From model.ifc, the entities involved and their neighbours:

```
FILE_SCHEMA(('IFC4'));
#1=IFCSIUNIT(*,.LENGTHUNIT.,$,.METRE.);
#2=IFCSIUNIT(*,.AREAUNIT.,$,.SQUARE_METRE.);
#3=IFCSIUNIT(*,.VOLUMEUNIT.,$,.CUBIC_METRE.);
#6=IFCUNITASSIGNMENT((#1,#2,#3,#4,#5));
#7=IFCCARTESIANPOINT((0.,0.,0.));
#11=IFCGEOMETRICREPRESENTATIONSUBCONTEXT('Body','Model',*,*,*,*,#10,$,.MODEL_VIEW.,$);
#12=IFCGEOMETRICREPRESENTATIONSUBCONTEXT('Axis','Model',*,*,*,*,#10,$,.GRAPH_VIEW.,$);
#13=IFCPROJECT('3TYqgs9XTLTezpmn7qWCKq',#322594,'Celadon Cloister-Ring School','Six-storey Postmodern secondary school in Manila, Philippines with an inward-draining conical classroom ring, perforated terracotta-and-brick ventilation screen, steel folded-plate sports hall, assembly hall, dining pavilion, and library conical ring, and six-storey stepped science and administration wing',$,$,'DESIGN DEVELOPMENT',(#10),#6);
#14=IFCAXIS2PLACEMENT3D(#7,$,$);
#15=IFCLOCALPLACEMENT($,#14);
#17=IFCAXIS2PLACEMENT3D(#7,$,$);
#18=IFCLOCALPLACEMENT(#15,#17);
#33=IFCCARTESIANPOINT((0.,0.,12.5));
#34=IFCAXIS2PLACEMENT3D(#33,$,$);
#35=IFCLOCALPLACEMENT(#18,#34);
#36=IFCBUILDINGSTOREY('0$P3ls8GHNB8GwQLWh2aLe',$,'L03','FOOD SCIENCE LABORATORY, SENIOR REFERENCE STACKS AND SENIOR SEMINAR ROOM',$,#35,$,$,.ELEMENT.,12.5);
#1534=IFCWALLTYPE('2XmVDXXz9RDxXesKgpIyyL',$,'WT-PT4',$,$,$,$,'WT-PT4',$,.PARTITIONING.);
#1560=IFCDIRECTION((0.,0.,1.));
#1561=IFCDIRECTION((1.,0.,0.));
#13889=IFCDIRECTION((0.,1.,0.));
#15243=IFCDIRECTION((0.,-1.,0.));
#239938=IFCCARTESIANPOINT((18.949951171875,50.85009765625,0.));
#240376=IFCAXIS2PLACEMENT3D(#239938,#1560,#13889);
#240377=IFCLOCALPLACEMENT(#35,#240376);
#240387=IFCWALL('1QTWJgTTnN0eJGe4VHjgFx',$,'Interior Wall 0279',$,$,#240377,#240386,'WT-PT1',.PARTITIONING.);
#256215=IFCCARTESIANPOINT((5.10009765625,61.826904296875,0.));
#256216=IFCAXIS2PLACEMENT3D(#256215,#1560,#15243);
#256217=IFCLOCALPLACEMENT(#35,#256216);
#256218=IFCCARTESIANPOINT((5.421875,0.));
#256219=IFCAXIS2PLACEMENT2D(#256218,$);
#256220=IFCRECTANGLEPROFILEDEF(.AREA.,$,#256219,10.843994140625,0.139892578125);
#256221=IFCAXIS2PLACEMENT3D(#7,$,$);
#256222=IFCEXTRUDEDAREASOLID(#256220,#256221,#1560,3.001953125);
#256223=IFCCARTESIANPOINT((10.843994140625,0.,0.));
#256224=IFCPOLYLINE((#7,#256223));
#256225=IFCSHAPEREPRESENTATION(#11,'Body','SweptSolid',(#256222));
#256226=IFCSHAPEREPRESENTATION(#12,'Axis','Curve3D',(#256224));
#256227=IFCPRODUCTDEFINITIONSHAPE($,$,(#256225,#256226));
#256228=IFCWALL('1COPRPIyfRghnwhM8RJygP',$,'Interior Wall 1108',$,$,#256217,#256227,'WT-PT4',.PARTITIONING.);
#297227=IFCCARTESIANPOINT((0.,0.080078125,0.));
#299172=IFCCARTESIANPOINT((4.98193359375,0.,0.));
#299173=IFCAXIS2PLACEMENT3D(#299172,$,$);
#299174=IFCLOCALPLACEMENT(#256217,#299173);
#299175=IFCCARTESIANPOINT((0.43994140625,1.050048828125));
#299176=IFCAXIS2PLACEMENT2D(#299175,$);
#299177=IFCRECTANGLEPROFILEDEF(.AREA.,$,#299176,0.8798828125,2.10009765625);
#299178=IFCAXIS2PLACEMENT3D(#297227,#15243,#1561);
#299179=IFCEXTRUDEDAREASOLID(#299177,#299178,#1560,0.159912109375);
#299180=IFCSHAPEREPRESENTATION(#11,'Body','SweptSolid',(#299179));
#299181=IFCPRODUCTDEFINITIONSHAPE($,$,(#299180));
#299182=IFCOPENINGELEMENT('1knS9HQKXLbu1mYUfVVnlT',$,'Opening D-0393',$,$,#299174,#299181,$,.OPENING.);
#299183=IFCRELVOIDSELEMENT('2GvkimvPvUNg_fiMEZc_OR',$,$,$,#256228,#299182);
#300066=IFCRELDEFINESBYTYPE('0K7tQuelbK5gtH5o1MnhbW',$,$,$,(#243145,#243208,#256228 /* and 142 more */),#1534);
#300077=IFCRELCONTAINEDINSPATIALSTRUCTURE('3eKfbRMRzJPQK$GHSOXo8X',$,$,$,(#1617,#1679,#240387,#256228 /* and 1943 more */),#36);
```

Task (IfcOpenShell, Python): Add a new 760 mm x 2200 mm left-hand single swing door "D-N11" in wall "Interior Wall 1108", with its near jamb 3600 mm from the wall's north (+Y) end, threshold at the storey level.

```python
import numpy as np
import ifcopenshell
import ifcopenshell.api.feature
import ifcopenshell.api.geometry
import ifcopenshell.api.root
import ifcopenshell.api.spatial
import ifcopenshell.geom
import ifcopenshell.util.element
import ifcopenshell.util.placement
import ifcopenshell.util.representation
import ifcopenshell.util.shape
import ifcopenshell.util.unit

model = ifcopenshell.open("model.ifc")
unit_scale = ifcopenshell.util.unit.calculate_unit_scale(model)
settings = ifcopenshell.geom.settings()


def volume(element):
    """Net volume in cubic metres, openings subtracted."""
    shape = ifcopenshell.geom.create_shape(settings, element)
    return ifcopenshell.util.shape.get_volume(shape.geometry)


wall = model.by_guid("1COPRPIyfRghnwhM8RJygP")
storey = ifcopenshell.util.element.get_container(wall, ifc_class="IfcBuildingStorey")
context = ifcopenshell.util.representation.get_context(model, "Model", "Body", "MODEL_VIEW")
before = volume(wall)

width, height, from_end, sill = 0.76, 2.2, 3.6, 0.0  # metres

# The wall runs along its own X axis, and the end named is its -X end.
wall_shape = ifcopenshell.geom.create_shape(settings, wall)
x, y, z = ifcopenshell.util.shape.get_vertices(wall_shape.geometry).T
start = x.min() + from_end
face, thickness = float(y.min()), float(y.max() - y.min())
wall_matrix = ifcopenshell.util.placement.get_local_placement(wall.ObjectPlacement)
level = ifcopenshell.util.placement.get_local_placement(storey.ObjectPlacement)[2, 3]


def in_wall(x, y):
    """Placement at x, y metres in the wall's axes, at sill height."""
    matrix = wall_matrix.copy()
    matrix[:, 3] = wall_matrix @ np.array([x / unit_scale, y / unit_scale, 0.0, 1.0])
    matrix[2, 3] = level + sill / unit_scale
    return matrix


# Opening: a box that overshoots both wall faces by 50 mm.
opening = ifcopenshell.api.root.create_entity(model, ifc_class="IfcOpeningElement", predefined_type="OPENING")
box = ifcopenshell.api.geometry.add_wall_representation(
    model, context=context, length=width, height=height, thickness=thickness + 0.1
)
ifcopenshell.api.geometry.assign_representation(model, product=opening, representation=box)
ifcopenshell.api.geometry.edit_object_placement(model, product=opening, matrix=in_wall(start, face - 0.05), is_si=False)
ifcopenshell.api.feature.add_feature(model, feature=opening, element=wall)

door = ifcopenshell.api.root.create_entity(model, ifc_class="IfcDoor", name="D-N11", predefined_type="DOOR")
door.OverallWidth, door.OverallHeight = width / unit_scale, height / unit_scale
door.OperationType = "SINGLE_SWING_LEFT"
body = ifcopenshell.api.geometry.add_door_representation(
    model,
    context=context,
    overall_width=door.OverallWidth,
    overall_height=door.OverallHeight,
    operation_type="SINGLE_SWING_LEFT",
    lining_properties={"LiningDepth": thickness / unit_scale, "ThresholdDepth": thickness / unit_scale},
)
ifcopenshell.api.geometry.assign_representation(model, product=door, representation=body)
ifcopenshell.api.spatial.assign_container(model, products=[door], relating_structure=storey)
ifcopenshell.api.feature.add_filling(model, opening=opening, element=door)

# The lining spans the wall, so the door starts at the wall face.
ifcopenshell.api.geometry.edit_object_placement(model, product=door, matrix=in_wall(start, face), is_si=False)

after = volume(wall)

print(f"wall volume {before:.3f} -> {after:.3f} m3")

model.write("model_rev.ifc")
```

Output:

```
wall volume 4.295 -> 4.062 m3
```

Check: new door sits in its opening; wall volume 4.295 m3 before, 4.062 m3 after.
